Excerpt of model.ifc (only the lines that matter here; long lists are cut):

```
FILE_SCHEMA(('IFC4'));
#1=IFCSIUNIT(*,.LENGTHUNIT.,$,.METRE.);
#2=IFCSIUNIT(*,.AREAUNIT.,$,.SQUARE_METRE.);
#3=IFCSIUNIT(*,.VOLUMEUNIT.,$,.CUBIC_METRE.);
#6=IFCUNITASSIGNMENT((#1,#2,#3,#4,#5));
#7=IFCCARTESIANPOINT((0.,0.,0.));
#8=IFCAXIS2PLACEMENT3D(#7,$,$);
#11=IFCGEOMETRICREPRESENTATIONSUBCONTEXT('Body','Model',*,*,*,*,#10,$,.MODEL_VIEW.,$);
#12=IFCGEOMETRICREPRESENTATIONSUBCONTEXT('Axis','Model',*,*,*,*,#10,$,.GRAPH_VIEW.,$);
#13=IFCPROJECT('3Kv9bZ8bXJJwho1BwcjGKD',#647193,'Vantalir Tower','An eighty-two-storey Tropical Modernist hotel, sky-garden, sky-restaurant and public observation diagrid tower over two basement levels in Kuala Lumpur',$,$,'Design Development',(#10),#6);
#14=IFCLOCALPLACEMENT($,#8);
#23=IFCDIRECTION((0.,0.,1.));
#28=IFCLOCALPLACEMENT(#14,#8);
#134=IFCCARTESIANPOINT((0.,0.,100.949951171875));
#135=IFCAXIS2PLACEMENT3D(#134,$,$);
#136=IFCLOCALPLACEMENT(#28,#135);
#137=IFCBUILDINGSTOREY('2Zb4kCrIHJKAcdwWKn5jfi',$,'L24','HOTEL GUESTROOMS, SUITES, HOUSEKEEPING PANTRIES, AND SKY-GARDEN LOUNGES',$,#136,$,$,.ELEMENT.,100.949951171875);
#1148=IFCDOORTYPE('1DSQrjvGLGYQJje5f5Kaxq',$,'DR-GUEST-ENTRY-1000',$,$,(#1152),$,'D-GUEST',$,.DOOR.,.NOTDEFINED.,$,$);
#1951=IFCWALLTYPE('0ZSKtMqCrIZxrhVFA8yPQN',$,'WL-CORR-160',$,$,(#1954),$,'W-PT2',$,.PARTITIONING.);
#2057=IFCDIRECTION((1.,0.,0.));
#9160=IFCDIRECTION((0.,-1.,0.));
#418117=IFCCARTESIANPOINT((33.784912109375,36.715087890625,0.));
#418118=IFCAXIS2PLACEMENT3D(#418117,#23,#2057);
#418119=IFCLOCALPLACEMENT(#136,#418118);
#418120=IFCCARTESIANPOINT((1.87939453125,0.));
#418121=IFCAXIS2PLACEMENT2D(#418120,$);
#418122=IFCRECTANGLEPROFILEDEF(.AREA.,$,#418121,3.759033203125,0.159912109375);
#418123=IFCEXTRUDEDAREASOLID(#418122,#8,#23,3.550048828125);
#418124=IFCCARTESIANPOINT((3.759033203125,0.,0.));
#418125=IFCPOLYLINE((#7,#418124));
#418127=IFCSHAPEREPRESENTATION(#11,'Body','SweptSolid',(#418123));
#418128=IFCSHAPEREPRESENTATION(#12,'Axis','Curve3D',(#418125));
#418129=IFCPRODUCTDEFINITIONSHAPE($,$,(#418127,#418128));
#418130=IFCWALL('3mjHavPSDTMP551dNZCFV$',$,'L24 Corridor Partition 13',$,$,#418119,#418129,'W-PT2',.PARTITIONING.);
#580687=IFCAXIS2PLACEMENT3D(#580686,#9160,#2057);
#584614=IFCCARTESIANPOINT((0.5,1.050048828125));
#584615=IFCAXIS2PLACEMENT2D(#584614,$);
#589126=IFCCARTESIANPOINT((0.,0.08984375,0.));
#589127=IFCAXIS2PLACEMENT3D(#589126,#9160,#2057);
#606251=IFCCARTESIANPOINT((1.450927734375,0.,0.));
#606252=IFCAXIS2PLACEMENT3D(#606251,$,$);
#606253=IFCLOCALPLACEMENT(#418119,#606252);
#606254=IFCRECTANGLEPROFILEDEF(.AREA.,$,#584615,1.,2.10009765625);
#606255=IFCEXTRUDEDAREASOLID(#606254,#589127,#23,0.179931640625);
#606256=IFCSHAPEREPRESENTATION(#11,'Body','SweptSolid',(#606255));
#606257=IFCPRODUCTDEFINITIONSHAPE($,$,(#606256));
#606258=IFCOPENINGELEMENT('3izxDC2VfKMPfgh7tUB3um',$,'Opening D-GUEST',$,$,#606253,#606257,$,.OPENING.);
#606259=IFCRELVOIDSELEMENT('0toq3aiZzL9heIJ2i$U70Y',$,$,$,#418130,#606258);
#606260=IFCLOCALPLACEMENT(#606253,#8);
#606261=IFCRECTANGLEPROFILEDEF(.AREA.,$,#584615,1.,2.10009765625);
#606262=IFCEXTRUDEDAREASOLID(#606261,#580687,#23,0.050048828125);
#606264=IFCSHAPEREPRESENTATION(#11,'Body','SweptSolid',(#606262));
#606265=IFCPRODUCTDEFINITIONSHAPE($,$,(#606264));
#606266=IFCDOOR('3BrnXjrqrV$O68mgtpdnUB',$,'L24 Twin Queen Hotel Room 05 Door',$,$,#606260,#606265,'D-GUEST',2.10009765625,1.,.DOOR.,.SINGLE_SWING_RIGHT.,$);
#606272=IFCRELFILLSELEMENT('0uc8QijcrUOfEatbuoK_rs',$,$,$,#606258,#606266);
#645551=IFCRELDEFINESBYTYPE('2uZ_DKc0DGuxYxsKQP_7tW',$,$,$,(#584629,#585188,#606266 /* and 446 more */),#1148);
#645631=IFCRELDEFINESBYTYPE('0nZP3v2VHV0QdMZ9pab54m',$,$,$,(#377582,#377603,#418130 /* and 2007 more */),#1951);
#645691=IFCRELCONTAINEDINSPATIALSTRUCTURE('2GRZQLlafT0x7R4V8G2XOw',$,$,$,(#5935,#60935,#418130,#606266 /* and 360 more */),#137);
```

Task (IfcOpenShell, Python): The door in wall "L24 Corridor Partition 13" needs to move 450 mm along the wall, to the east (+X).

```python
import ifcopenshell
import ifcopenshell.api.geometry
import ifcopenshell.util.placement

model = ifcopenshell.open("model.ifc")

door = model.by_id(606266)
opening = door.FillsVoids[0].RelatingOpeningElement
wall = opening.VoidsElements[0].RelatingBuildingElement

wall_matrix = ifcopenshell.util.placement.get_local_placement(wall.ObjectPlacement)
shift = wall_matrix[:3, 0] * 0.45
before = ifcopenshell.util.placement.get_local_placement(door.ObjectPlacement)[:3, 3].copy()

# The door is placed relative to its opening, so it follows when the opening moves.
matrix = ifcopenshell.util.placement.get_local_placement(opening.ObjectPlacement)
matrix[:3, 3] += shift
ifcopenshell.api.geometry.edit_object_placement(
    model, product=opening, matrix=matrix, is_si=False, should_transform_children=True
)

after = ifcopenshell.util.placement.get_local_placement(door.ObjectPlacement)[:3, 3]
print("door moved by", (after - before).round(3) + 0.0)

model.write("model_rev.ifc")
```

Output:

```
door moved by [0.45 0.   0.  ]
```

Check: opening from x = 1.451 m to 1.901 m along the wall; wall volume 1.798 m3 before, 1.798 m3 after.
